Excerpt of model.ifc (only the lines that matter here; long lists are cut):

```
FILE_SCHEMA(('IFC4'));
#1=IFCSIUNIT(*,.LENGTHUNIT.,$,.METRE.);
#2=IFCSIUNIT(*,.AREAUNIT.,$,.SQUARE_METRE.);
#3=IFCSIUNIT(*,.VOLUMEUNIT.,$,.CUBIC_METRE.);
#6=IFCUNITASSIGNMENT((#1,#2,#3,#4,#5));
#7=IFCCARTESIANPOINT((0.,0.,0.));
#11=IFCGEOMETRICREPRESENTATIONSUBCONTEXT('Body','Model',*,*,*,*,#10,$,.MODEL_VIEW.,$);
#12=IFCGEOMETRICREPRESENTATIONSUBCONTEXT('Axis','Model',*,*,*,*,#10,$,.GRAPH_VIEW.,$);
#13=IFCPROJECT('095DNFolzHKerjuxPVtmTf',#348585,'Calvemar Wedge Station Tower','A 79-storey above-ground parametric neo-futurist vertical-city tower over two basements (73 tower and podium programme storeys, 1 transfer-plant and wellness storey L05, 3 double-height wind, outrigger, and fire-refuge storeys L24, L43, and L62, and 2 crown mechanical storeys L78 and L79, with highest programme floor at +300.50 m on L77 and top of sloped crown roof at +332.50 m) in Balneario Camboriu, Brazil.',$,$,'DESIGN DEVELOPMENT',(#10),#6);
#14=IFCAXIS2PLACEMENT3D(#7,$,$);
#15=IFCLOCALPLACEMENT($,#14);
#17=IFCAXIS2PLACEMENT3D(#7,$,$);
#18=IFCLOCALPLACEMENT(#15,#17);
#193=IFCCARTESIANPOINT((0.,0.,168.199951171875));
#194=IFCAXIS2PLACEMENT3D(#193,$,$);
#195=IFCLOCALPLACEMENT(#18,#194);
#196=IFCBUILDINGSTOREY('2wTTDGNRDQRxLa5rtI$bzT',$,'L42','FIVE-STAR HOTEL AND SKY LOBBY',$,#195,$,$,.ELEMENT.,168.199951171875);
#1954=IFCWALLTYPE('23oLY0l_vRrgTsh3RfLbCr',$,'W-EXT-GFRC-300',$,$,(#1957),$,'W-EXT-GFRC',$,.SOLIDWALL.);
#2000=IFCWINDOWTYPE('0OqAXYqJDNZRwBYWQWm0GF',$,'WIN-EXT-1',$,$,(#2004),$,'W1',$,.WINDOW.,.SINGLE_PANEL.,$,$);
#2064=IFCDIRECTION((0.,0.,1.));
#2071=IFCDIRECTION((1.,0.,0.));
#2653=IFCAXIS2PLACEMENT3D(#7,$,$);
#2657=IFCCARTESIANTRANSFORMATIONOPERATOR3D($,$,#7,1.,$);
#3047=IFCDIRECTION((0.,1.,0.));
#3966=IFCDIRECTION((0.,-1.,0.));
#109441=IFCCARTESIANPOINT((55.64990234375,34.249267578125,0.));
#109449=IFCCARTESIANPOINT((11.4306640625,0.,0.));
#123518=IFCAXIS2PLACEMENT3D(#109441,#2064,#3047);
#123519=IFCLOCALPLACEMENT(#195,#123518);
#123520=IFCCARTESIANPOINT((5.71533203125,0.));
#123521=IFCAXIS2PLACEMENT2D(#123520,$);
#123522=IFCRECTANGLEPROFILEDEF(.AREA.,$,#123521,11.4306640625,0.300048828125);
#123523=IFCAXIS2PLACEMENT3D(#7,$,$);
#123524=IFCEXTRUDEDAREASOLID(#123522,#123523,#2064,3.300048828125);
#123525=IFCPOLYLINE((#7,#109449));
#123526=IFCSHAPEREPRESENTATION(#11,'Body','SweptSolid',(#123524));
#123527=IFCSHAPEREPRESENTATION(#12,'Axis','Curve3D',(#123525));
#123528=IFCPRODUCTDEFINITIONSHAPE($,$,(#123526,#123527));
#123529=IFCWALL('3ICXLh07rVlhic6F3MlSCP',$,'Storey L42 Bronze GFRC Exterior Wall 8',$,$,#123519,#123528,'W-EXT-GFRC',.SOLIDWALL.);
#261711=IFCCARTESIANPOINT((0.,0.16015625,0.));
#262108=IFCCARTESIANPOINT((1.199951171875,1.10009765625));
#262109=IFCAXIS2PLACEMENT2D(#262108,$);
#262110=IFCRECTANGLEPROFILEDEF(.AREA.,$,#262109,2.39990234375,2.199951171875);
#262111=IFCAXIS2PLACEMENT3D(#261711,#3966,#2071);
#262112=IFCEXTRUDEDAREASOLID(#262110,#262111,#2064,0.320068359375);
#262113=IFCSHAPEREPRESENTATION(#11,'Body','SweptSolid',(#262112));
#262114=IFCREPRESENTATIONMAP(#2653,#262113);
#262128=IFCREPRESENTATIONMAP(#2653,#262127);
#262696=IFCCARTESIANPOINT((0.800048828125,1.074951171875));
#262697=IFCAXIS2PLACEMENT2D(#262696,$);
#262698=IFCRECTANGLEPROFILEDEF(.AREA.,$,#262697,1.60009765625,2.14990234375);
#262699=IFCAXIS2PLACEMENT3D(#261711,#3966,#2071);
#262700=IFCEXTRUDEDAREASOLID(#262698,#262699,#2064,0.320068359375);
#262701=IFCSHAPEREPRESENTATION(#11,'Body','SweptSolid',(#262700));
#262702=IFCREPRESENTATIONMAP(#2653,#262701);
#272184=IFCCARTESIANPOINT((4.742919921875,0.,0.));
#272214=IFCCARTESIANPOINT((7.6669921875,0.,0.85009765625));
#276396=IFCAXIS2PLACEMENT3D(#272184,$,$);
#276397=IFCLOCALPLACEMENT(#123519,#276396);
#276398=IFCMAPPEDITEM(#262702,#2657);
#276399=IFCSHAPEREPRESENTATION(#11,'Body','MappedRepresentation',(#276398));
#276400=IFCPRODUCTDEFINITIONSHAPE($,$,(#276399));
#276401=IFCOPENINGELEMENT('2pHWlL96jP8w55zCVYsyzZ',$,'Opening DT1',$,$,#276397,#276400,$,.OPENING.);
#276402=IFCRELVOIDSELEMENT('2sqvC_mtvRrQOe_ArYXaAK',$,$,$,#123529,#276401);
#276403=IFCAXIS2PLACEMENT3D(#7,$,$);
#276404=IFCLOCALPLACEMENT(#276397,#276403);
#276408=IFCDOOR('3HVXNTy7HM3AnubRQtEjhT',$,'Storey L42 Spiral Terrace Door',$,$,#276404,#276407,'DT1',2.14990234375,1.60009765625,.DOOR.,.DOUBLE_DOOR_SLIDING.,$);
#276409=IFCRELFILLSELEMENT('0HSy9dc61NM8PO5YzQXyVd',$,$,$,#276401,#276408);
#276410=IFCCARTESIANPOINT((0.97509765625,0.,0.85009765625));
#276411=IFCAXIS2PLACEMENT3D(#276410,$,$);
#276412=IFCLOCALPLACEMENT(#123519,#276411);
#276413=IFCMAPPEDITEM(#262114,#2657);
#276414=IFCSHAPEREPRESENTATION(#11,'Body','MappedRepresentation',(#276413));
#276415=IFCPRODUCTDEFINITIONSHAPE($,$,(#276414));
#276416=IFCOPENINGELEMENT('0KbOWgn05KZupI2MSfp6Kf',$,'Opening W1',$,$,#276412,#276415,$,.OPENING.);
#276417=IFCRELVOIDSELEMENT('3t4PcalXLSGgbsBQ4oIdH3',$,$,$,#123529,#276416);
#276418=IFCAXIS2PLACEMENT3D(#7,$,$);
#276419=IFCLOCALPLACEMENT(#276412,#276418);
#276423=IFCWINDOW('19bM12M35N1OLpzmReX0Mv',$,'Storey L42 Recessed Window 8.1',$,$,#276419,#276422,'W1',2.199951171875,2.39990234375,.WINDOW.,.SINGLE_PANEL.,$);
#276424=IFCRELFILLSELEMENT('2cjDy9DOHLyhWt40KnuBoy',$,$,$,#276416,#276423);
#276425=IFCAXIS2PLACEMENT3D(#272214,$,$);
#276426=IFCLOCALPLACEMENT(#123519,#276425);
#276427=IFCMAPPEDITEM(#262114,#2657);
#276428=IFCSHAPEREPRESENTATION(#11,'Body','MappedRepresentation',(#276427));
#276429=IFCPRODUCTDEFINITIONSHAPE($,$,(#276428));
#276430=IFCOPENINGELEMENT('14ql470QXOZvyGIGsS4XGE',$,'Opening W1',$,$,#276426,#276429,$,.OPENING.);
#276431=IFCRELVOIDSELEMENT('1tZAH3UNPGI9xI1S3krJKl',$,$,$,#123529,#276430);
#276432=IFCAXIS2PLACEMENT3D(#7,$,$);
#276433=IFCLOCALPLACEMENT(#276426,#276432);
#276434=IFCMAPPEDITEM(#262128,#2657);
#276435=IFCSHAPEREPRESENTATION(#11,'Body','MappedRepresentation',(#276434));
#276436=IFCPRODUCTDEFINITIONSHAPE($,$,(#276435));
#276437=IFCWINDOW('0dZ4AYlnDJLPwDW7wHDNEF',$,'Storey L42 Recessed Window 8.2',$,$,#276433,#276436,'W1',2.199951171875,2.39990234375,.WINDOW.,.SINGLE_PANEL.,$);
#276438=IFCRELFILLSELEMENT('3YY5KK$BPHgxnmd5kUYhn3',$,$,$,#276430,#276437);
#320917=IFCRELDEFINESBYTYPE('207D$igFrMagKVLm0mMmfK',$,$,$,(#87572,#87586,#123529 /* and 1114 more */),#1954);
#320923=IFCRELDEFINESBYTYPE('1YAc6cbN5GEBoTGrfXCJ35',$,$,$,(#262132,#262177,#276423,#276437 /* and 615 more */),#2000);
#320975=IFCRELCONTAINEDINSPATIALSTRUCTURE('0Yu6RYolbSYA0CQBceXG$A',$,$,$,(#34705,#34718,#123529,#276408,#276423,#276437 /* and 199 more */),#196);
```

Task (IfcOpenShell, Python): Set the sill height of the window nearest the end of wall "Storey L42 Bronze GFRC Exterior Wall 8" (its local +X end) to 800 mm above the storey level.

```python
import numpy as np
import ifcopenshell
import ifcopenshell.api.geometry
import ifcopenshell.geom
import ifcopenshell.util.element
import ifcopenshell.util.placement
import ifcopenshell.util.shape
import ifcopenshell.util.unit

model = ifcopenshell.open("model.ifc")
unit_scale = ifcopenshell.util.unit.calculate_unit_scale(model)

window = model.by_guid("0dZ4AYlnDJLPwDW7wHDNEF")
opening = window.FillsVoids[0].RelatingOpeningElement
storey = ifcopenshell.util.element.get_container(window, ifc_class="IfcBuildingStorey")
level = ifcopenshell.util.placement.get_local_placement(storey.ObjectPlacement)[2, 3]

# The opening's origin need not be at the sill, so measure its lowest point.
shape = ifcopenshell.geom.create_shape(ifcopenshell.geom.settings(), opening)
bottom = ifcopenshell.util.shape.get_shape_bottom_elevation(shape, shape.geometry) / unit_scale
dz = level + 0.8 / unit_scale - bottom

shift = np.array([0.0, 0.0, dz])
# The window is placed relative to its opening, so it follows when the opening moves.
matrix = ifcopenshell.util.placement.get_local_placement(opening.ObjectPlacement)
matrix[:3, 3] += shift
ifcopenshell.api.geometry.edit_object_placement(
    model, product=opening, matrix=matrix, is_si=False, should_transform_children=True
)

print(f"moved by {dz * unit_scale:+.3f} m")

model.write("model_v2.ifc")
```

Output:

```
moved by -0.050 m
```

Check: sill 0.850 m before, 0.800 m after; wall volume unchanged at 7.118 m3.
